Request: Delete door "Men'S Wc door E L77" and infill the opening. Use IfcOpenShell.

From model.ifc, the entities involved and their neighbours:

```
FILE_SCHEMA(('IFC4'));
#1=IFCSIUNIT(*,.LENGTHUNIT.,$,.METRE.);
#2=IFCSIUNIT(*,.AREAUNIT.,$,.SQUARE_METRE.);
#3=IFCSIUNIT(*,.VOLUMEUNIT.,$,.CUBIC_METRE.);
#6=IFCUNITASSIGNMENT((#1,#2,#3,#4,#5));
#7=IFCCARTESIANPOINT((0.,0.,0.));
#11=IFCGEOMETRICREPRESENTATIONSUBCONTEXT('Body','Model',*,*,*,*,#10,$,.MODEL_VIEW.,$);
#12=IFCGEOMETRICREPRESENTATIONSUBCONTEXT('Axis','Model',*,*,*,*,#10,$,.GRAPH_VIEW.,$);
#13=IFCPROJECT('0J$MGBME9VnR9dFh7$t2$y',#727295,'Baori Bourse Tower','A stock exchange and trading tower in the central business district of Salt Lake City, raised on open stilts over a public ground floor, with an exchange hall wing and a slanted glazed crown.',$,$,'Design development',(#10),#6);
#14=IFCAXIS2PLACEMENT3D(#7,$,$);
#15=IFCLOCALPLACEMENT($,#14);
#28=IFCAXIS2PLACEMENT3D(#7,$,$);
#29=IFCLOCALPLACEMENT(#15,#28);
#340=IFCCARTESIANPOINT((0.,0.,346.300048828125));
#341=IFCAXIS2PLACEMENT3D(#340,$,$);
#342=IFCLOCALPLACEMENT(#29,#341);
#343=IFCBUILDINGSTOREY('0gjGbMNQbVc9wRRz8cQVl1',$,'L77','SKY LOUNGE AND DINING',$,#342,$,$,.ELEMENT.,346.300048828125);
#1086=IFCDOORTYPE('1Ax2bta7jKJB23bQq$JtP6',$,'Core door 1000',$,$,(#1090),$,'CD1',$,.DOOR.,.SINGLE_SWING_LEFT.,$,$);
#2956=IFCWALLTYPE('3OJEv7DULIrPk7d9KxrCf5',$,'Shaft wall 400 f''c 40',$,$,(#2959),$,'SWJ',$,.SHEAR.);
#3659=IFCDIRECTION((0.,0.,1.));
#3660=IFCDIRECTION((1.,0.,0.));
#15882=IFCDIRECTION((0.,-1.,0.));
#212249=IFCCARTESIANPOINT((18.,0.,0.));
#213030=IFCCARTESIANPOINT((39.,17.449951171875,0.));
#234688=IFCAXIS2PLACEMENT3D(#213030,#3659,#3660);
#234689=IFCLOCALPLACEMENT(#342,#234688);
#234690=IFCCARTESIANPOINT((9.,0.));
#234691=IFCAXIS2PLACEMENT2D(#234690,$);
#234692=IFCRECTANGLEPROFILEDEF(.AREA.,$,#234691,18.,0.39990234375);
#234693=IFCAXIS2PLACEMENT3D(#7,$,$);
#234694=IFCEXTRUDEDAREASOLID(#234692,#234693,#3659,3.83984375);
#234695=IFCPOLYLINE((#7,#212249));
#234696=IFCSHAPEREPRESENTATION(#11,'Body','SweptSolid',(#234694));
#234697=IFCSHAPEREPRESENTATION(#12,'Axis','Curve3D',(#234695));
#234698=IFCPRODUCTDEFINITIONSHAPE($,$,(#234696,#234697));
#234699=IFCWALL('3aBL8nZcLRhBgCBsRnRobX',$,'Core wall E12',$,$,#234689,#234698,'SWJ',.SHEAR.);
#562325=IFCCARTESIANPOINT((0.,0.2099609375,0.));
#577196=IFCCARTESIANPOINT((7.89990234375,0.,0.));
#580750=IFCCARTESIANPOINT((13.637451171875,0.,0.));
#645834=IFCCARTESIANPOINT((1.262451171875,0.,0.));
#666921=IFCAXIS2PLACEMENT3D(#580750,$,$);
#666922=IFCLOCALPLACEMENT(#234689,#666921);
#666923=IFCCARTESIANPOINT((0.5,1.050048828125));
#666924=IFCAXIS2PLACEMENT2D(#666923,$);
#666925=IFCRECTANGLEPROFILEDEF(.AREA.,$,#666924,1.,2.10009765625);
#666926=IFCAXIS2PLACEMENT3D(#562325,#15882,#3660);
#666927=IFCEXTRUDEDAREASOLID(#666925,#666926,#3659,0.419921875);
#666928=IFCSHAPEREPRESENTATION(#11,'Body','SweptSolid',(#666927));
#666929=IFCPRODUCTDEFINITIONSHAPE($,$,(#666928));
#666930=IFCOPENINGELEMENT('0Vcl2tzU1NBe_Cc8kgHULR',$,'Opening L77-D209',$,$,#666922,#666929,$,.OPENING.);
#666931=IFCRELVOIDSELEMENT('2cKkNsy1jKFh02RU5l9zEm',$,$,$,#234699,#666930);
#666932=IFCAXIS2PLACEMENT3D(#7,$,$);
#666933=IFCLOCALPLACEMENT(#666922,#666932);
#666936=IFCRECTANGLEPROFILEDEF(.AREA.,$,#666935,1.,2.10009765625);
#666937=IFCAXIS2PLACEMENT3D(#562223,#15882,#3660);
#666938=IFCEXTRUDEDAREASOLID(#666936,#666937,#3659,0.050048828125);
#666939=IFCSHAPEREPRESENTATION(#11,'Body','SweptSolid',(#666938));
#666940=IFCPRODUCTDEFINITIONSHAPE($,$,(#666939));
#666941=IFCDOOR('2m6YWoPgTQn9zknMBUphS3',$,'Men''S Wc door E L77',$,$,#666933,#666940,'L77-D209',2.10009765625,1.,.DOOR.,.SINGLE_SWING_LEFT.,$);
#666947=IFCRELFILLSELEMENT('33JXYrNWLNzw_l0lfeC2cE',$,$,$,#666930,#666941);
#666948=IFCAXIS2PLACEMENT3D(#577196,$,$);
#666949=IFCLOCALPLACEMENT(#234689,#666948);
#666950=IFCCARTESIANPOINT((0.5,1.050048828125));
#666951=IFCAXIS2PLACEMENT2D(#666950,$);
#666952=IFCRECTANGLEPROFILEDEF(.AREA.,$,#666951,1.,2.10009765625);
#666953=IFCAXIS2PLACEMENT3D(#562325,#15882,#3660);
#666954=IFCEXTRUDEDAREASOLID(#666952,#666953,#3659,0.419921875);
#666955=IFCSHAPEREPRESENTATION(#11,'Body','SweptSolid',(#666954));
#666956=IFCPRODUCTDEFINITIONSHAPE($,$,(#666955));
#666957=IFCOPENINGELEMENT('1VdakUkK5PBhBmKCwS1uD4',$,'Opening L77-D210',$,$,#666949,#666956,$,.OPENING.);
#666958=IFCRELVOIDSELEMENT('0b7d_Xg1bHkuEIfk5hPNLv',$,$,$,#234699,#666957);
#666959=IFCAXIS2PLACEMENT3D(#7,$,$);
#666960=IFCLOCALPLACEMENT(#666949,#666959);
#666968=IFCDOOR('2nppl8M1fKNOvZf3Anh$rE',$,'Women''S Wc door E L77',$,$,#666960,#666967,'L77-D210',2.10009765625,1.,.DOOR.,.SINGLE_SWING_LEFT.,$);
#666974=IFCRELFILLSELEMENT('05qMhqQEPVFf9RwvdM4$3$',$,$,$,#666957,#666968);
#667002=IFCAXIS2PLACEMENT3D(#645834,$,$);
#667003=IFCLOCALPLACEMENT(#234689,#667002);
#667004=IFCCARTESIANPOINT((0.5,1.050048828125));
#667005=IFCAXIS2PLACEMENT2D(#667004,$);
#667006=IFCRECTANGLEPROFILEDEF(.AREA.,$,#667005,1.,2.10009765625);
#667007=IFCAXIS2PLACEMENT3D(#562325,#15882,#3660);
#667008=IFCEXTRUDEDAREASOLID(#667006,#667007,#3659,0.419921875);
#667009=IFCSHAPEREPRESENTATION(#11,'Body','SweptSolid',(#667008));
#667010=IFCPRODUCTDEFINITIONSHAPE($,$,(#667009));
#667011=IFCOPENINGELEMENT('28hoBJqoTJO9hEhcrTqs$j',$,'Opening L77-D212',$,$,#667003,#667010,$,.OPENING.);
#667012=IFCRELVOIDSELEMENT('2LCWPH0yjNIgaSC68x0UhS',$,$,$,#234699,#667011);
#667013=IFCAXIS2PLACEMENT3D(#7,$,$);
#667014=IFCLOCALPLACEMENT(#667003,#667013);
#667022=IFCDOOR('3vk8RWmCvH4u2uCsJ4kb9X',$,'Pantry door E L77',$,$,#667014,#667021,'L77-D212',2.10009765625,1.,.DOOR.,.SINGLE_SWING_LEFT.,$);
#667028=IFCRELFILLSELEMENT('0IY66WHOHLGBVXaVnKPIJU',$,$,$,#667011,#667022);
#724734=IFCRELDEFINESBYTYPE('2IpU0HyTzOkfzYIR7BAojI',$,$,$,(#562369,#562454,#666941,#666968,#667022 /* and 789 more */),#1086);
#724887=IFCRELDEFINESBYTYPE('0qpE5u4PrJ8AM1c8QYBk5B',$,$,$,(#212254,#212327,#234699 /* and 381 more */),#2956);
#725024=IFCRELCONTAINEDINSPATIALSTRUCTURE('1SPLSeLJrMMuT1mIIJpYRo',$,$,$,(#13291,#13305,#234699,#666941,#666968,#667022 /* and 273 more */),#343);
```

```python
import ifcopenshell
import ifcopenshell.api.feature
import ifcopenshell.api.root
import ifcopenshell.geom
import ifcopenshell.util.shape

model = ifcopenshell.open("model.ifc")
settings = ifcopenshell.geom.settings()


def volume(element):
    """Net volume in cubic metres, openings subtracted."""
    shape = ifcopenshell.geom.create_shape(settings, element)
    return ifcopenshell.util.shape.get_volume(shape.geometry)


door = model.by_guid("2m6YWoPgTQn9zknMBUphS3")
opening = door.FillsVoids[0].RelatingOpeningElement
wall = opening.VoidsElements[0].RelatingBuildingElement
before = volume(wall)

ifcopenshell.api.root.remove_product(model, product=door)
ifcopenshell.api.feature.remove_feature(model, feature=opening)

after = volume(wall)

print(f"wall volume {before:.3f} -> {after:.3f} m3")

model.write("model-out.ifc")
```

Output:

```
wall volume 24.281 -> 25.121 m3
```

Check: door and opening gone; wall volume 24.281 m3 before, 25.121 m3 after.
